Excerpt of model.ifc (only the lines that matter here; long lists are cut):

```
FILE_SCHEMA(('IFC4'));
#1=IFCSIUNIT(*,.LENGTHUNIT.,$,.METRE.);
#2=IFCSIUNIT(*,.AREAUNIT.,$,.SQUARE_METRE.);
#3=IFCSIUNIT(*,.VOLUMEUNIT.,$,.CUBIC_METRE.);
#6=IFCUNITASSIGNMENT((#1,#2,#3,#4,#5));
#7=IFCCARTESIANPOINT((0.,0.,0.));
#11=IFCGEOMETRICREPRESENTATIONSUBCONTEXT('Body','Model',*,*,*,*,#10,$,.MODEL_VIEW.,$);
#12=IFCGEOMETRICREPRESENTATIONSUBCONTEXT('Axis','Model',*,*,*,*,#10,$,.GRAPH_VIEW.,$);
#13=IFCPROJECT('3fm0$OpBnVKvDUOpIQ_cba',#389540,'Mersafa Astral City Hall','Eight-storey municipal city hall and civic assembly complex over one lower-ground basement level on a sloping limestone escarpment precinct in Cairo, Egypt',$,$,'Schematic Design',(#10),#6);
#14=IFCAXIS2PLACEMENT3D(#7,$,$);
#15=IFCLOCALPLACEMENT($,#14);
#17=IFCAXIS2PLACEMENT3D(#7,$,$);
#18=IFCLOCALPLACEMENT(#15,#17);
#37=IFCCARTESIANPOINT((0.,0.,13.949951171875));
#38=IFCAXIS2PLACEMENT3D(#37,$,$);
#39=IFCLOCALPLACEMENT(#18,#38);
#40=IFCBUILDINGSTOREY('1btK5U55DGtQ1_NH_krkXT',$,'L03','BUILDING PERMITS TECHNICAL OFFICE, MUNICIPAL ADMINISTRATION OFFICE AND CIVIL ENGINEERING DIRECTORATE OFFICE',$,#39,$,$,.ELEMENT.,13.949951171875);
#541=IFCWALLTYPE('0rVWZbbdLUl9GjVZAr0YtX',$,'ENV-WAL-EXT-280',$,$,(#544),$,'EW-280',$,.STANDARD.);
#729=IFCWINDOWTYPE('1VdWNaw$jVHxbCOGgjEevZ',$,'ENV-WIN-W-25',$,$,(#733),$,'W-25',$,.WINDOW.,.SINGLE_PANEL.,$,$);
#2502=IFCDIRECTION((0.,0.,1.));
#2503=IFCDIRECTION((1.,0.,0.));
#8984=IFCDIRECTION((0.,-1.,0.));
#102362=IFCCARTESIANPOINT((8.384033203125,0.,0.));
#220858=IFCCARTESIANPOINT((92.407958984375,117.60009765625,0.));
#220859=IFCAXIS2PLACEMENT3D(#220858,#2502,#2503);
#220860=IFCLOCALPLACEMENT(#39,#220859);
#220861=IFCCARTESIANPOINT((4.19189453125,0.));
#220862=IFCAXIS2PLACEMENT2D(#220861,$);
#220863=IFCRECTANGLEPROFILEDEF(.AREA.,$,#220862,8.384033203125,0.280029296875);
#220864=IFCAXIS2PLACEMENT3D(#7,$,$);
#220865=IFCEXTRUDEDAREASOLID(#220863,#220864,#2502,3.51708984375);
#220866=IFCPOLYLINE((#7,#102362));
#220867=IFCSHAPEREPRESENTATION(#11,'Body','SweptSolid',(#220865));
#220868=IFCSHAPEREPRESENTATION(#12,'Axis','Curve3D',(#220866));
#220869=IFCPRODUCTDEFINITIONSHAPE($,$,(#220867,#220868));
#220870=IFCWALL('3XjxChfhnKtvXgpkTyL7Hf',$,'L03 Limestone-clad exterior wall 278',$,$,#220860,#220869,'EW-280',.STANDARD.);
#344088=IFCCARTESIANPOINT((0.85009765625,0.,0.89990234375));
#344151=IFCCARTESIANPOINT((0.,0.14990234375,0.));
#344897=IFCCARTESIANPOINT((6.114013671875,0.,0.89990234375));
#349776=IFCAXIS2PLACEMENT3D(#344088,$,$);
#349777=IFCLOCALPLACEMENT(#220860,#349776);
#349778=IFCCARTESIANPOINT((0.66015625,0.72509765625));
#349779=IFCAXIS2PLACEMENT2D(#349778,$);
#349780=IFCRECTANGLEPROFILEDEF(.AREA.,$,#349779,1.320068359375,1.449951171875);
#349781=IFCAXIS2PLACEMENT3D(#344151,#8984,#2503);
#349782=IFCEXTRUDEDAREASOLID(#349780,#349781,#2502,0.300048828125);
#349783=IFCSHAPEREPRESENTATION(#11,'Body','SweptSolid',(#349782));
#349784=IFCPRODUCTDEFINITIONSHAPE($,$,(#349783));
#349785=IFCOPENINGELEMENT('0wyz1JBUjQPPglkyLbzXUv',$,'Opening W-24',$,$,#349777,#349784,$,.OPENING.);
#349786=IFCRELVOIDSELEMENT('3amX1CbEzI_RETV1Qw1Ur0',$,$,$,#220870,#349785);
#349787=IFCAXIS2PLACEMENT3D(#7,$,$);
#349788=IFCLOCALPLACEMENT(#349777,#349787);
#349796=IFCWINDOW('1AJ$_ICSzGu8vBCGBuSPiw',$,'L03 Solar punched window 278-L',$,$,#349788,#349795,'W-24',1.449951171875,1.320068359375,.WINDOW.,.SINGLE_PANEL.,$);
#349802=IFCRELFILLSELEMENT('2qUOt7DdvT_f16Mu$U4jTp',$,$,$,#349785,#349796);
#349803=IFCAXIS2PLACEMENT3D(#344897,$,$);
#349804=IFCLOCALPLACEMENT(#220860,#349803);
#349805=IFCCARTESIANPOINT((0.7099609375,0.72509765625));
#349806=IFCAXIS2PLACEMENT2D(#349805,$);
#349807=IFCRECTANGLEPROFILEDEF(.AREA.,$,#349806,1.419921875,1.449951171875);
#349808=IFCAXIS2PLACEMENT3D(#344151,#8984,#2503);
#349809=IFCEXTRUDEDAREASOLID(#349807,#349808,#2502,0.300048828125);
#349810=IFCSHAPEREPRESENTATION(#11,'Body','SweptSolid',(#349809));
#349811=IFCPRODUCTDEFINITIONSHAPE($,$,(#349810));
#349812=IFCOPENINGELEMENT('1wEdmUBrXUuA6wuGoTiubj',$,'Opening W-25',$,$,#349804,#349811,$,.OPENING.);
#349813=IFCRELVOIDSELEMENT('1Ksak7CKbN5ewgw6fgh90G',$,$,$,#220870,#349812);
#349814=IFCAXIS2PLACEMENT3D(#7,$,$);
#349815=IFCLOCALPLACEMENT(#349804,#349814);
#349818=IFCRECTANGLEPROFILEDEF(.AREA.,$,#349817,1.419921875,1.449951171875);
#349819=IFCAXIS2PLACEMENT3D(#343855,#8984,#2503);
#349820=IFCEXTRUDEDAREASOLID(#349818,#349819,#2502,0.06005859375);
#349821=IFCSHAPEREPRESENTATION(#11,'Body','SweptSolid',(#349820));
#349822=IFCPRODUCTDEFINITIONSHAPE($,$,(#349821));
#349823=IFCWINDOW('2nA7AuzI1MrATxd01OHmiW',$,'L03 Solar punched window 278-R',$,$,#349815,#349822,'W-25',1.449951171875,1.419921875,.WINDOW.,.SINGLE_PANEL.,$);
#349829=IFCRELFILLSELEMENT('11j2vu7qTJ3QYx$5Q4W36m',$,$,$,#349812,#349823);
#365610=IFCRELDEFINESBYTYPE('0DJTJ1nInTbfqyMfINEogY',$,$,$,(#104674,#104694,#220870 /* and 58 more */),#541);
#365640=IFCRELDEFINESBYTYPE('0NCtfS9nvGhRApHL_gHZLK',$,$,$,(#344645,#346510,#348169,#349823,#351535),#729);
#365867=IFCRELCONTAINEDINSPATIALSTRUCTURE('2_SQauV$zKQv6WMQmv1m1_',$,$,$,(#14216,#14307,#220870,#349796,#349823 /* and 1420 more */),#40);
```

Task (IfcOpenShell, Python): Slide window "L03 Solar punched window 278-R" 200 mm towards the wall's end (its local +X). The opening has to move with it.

```python
import ifcopenshell
import ifcopenshell.api.geometry
import ifcopenshell.util.placement

model = ifcopenshell.open("model.ifc")

window = model.by_guid("2nA7AuzI1MrATxd01OHmiW")
opening = window.FillsVoids[0].RelatingOpeningElement
wall = opening.VoidsElements[0].RelatingBuildingElement

wall_matrix = ifcopenshell.util.placement.get_local_placement(wall.ObjectPlacement)
shift = wall_matrix[:3, 0] * 0.2
before = ifcopenshell.util.placement.get_local_placement(window.ObjectPlacement)[:3, 3].copy()

# The window is placed relative to its opening, so it follows when the opening moves.
matrix = ifcopenshell.util.placement.get_local_placement(opening.ObjectPlacement)
matrix[:3, 3] += shift
ifcopenshell.api.geometry.edit_object_placement(
    model, product=opening, matrix=matrix, is_si=False, should_transform_children=True
)

after = ifcopenshell.util.placement.get_local_placement(window.ObjectPlacement)[:3, 3]
print("window moved by", (after - before).round(3) + 0.0)

model.write("model_rev.ifc")
```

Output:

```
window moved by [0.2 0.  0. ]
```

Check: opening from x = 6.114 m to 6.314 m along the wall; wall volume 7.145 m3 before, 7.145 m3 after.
